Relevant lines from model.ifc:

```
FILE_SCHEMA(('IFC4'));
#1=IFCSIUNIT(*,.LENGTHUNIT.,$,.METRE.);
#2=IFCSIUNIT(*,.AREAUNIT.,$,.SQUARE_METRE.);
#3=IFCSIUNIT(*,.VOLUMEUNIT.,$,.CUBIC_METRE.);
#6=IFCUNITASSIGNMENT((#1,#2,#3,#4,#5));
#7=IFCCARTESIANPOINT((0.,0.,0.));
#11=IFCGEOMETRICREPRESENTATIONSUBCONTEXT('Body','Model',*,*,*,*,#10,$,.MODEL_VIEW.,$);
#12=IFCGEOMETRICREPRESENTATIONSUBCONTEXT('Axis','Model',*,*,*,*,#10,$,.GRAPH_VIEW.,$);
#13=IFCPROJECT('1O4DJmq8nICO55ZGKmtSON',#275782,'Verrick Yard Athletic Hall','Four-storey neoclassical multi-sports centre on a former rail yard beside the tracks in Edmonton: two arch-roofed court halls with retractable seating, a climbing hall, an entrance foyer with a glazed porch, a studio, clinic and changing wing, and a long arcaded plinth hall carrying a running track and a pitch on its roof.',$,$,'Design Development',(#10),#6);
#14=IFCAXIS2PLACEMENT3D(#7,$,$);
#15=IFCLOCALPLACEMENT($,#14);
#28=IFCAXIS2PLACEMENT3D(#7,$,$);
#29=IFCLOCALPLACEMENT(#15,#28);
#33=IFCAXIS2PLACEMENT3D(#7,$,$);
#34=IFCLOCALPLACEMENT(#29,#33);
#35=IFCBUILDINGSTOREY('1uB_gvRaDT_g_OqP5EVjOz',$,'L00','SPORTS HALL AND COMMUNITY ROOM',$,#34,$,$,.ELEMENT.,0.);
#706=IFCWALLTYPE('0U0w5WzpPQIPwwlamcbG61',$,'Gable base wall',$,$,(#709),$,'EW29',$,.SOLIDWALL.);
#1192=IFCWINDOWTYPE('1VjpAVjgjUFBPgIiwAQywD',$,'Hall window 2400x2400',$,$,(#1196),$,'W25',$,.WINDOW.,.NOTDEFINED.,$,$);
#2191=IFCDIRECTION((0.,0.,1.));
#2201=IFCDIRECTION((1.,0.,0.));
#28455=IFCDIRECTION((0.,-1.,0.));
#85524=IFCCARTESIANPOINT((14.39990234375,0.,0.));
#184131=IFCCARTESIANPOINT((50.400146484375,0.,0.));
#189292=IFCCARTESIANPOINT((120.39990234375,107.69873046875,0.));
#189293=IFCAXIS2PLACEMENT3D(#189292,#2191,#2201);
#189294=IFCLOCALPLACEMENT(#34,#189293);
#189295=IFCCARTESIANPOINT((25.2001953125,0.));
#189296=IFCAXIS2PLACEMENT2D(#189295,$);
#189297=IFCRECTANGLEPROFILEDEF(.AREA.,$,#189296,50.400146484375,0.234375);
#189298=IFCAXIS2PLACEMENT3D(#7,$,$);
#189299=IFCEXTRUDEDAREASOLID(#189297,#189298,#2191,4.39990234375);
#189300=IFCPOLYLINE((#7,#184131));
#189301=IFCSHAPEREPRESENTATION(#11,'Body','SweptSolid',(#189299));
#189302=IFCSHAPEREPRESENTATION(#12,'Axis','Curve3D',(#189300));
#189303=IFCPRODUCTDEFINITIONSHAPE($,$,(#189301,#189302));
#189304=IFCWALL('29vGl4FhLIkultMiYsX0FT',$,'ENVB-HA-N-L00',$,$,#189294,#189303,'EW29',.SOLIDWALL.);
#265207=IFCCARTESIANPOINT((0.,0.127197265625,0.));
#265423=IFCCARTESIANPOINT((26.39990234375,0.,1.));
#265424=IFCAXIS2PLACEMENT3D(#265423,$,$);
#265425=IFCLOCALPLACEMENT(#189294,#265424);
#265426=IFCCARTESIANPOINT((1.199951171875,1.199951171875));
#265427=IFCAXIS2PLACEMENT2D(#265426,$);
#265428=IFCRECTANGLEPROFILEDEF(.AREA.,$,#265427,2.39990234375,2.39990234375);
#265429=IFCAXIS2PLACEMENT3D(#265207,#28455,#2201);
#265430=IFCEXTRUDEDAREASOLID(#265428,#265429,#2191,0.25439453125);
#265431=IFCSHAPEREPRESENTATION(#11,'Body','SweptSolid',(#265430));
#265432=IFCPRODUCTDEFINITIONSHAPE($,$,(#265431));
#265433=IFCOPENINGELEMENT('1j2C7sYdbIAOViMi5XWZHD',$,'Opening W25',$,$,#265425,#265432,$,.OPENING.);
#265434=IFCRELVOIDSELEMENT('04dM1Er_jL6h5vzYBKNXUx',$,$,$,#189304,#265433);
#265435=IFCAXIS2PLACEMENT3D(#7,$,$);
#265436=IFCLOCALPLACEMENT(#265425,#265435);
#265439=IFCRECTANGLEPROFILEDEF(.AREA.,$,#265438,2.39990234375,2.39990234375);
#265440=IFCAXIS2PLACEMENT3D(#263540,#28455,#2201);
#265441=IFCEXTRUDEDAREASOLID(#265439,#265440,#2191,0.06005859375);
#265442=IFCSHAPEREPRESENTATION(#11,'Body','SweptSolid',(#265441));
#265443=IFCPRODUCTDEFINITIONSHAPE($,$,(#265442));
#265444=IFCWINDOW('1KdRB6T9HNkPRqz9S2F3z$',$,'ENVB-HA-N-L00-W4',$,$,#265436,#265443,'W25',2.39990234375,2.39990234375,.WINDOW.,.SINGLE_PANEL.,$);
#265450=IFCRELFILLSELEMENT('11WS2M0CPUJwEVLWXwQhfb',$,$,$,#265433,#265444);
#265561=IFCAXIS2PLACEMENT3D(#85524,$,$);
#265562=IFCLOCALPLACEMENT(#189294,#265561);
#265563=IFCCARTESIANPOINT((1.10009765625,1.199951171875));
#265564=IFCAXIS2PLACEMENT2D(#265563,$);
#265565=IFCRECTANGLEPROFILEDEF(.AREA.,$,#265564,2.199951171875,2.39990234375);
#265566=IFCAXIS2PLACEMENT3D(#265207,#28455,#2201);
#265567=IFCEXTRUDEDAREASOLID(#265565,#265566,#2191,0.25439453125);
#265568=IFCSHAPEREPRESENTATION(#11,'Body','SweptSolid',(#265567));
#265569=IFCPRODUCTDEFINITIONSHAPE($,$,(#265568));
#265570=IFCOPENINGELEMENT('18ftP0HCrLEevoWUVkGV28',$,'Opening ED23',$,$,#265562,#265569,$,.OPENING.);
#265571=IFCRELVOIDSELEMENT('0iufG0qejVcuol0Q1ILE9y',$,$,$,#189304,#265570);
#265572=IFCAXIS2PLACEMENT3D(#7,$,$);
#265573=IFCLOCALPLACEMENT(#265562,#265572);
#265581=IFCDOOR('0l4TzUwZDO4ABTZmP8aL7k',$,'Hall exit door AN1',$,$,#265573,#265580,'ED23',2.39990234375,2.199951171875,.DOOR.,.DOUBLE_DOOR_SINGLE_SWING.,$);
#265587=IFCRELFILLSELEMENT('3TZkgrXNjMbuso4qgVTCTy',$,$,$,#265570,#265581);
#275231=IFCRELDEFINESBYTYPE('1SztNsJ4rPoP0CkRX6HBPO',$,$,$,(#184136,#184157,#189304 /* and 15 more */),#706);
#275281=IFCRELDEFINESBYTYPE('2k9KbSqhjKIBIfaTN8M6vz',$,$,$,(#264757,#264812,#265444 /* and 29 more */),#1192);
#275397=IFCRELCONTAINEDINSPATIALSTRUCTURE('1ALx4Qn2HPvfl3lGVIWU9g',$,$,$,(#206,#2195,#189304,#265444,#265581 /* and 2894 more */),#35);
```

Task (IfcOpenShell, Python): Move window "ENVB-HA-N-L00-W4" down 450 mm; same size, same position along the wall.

```python
import numpy as np
import ifcopenshell
import ifcopenshell.api.geometry
import ifcopenshell.util.placement
import ifcopenshell.util.unit

model = ifcopenshell.open("model.ifc")
unit_scale = ifcopenshell.util.unit.calculate_unit_scale(model)

window = model.by_guid("1KdRB6T9HNkPRqz9S2F3z$")
opening = window.FillsVoids[0].RelatingOpeningElement
dz = -0.45 / unit_scale

shift = np.array([0.0, 0.0, dz])
# The window is placed relative to its opening, so it follows when the opening moves.
matrix = ifcopenshell.util.placement.get_local_placement(opening.ObjectPlacement)
matrix[:3, 3] += shift
ifcopenshell.api.geometry.edit_object_placement(
    model, product=opening, matrix=matrix, is_si=False, should_transform_children=True
)

print(f"moved by {dz * unit_scale:+.3f} m")

model.write("model_updated.ifc")
```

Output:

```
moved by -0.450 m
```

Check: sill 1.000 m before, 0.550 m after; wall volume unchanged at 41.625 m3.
